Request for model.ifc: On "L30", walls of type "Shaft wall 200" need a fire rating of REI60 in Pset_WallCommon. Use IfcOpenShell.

First a look at what the model holds.

```python
import ifcopenshell
import ifcopenshell.util.element

model = ifcopenshell.open("model.ifc")
print(model.schema)
storey = next(s for s in model.by_type("IfcBuildingStorey") if s.Name == "L30")
walls = [e for e in ifcopenshell.util.element.get_decomposition(storey) if e.is_a("IfcWall")]
seen = {}
for e in walls:
    element_type = ifcopenshell.util.element.get_type(e)
    key = (element_type.Name if element_type != e and element_type else None, ifcopenshell.util.element.get_pset(e, "Pset_WallCommon", "FireRating"))
    seen[key] = seen.get(key, 0) + 1
for (name, value), count in sorted(seen.items(), key=str):
    print(count, "x", name, "|", value)
```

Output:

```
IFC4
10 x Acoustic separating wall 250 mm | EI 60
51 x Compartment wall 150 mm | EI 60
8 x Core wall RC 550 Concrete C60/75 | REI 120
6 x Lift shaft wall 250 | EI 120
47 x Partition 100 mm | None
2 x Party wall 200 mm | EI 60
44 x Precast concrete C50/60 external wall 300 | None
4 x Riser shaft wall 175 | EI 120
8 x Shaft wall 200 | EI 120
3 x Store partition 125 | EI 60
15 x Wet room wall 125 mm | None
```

```python
import ifcopenshell
import ifcopenshell.api.pset
import ifcopenshell.util.element

model = ifcopenshell.open("model.ifc")

storey = next(s for s in model.by_type("IfcBuildingStorey") if s.Name == "L30")
walls = [e for e in ifcopenshell.util.element.get_decomposition(storey) if e.is_a("IfcWall")]

count = 0
for e in walls:
    element_type = ifcopenshell.util.element.get_type(e)
    if element_type in (None, e) or element_type.Name != "Shaft wall 200":
        continue
    found = ifcopenshell.util.element.get_pset(e, "Pset_WallCommon", should_inherit=False)
    if found:
        pset = model.by_id(found["id"])
        if len(ifcopenshell.util.element.get_elements_by_pset(pset)) > 1:
            pset = ifcopenshell.api.pset.unshare_pset(model, products=[e], pset=pset)[0]
    else:
        pset = ifcopenshell.api.pset.add_pset(model, product=e, name="Pset_WallCommon")
    ifcopenshell.api.pset.edit_pset(model, pset=pset, properties={"FireRating": "REI60"})
    count += 1

print(count, "walls updated")

model.write("model_edited.ifc")
```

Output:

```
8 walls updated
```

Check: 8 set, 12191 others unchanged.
